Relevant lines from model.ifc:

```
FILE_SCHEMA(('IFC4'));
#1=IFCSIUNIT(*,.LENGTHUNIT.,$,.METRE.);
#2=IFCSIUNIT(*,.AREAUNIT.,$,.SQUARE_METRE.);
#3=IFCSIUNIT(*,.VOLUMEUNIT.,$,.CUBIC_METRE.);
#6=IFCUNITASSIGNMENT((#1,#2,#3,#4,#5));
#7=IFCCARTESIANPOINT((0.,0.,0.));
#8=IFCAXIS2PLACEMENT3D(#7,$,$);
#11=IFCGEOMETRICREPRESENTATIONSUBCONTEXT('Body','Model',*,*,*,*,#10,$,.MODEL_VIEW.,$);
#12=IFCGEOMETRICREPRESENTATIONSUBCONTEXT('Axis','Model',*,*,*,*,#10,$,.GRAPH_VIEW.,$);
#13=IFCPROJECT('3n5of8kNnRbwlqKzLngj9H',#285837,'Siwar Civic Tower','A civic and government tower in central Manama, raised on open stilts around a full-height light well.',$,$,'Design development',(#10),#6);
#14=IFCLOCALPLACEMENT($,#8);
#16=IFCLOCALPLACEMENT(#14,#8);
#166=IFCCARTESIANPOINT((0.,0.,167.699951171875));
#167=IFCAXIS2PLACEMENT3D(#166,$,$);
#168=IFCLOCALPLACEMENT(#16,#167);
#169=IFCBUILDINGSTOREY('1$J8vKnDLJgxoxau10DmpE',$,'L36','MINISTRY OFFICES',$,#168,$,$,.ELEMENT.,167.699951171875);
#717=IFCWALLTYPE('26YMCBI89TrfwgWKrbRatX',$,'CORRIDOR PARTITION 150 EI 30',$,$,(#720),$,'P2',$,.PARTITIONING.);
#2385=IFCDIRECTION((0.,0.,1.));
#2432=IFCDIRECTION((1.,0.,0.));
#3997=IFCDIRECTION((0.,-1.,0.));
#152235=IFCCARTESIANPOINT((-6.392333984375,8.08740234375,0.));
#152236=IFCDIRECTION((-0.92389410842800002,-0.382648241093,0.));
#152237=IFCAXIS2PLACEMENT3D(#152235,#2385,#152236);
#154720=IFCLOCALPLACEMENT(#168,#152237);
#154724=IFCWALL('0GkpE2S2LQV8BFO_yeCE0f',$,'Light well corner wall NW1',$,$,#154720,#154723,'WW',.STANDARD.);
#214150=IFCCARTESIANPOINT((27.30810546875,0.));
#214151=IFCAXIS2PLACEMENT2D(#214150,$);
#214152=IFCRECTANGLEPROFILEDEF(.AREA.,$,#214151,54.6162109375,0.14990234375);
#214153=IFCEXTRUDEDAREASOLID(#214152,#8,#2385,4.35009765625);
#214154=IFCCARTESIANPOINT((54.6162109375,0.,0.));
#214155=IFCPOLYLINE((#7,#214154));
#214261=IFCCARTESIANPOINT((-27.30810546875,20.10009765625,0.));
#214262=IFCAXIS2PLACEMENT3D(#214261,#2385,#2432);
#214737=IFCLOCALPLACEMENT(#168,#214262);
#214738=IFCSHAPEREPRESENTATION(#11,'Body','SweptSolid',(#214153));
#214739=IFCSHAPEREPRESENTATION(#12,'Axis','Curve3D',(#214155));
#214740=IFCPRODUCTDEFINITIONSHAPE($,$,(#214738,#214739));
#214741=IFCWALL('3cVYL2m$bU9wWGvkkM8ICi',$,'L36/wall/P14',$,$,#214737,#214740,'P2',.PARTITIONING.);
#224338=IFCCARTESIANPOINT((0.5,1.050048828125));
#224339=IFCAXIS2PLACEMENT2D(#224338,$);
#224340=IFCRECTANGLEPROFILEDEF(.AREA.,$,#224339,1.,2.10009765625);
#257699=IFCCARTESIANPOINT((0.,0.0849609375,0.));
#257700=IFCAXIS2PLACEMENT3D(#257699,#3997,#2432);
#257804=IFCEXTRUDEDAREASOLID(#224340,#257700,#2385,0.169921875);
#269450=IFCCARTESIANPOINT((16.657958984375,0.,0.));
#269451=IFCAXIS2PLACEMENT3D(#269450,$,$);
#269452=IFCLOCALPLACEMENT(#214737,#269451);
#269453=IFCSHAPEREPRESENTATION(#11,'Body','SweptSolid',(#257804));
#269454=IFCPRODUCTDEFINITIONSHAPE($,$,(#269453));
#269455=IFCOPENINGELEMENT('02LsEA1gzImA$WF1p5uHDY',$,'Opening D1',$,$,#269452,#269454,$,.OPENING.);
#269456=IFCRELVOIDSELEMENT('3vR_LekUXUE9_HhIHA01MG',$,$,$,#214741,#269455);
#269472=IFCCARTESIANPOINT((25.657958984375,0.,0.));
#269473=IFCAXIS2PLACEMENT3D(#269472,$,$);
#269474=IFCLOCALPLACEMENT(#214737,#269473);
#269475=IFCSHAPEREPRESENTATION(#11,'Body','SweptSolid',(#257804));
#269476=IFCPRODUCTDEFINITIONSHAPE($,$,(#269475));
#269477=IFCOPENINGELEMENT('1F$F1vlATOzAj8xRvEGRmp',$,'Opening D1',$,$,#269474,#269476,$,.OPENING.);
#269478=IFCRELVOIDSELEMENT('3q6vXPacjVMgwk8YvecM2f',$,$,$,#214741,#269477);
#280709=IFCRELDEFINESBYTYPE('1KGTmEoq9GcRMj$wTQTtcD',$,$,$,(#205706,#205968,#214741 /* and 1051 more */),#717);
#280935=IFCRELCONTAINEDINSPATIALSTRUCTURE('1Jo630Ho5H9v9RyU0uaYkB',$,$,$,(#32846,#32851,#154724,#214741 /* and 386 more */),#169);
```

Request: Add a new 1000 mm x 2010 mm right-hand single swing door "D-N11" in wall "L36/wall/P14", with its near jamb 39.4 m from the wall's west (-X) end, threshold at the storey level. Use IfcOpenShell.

```python
import numpy as np
import ifcopenshell
import ifcopenshell.api.feature
import ifcopenshell.api.geometry
import ifcopenshell.api.root
import ifcopenshell.api.spatial
import ifcopenshell.geom
import ifcopenshell.util.element
import ifcopenshell.util.placement
import ifcopenshell.util.representation
import ifcopenshell.util.shape
import ifcopenshell.util.unit

model = ifcopenshell.open("model.ifc")
unit_scale = ifcopenshell.util.unit.calculate_unit_scale(model)
settings = ifcopenshell.geom.settings()


def volume(element):
    """Net volume in cubic metres, openings subtracted."""
    shape = ifcopenshell.geom.create_shape(settings, element)
    return ifcopenshell.util.shape.get_volume(shape.geometry)


wall = model.by_guid("3cVYL2m$bU9wWGvkkM8ICi")
storey = ifcopenshell.util.element.get_container(wall, ifc_class="IfcBuildingStorey")
context = ifcopenshell.util.representation.get_context(model, "Model", "Body", "MODEL_VIEW")
before = volume(wall)

width, height, from_end, sill = 1, 2.01, 39.4, 0.0  # metres

# The wall runs along its own X axis, and the end named is its -X end.
wall_shape = ifcopenshell.geom.create_shape(settings, wall)
x, y, z = ifcopenshell.util.shape.get_vertices(wall_shape.geometry).T
start = x.min() + from_end
face, thickness = float(y.min()), float(y.max() - y.min())
wall_matrix = ifcopenshell.util.placement.get_local_placement(wall.ObjectPlacement)
level = ifcopenshell.util.placement.get_local_placement(storey.ObjectPlacement)[2, 3]


def in_wall(x, y):
    """Placement at x, y metres in the wall's axes, at sill height."""
    matrix = wall_matrix.copy()
    matrix[:, 3] = wall_matrix @ np.array([x / unit_scale, y / unit_scale, 0.0, 1.0])
    matrix[2, 3] = level + sill / unit_scale
    return matrix


# Opening: a box that overshoots both wall faces by 50 mm.
opening = ifcopenshell.api.root.create_entity(model, ifc_class="IfcOpeningElement", predefined_type="OPENING")
box = ifcopenshell.api.geometry.add_wall_representation(
    model, context=context, length=width, height=height, thickness=thickness + 0.1
)
ifcopenshell.api.geometry.assign_representation(model, product=opening, representation=box)
ifcopenshell.api.geometry.edit_object_placement(model, product=opening, matrix=in_wall(start, face - 0.05), is_si=False)
ifcopenshell.api.feature.add_feature(model, feature=opening, element=wall)

door = ifcopenshell.api.root.create_entity(model, ifc_class="IfcDoor", name="D-N11", predefined_type="DOOR")
door.OverallWidth, door.OverallHeight = width / unit_scale, height / unit_scale
door.OperationType = "SINGLE_SWING_RIGHT"
body = ifcopenshell.api.geometry.add_door_representation(
    model,
    context=context,
    overall_width=door.OverallWidth,
    overall_height=door.OverallHeight,
    operation_type="SINGLE_SWING_RIGHT",
    lining_properties={"LiningDepth": thickness / unit_scale, "ThresholdDepth": thickness / unit_scale},
)
ifcopenshell.api.geometry.assign_representation(model, product=door, representation=body)
ifcopenshell.api.spatial.assign_container(model, products=[door], relating_structure=storey)
ifcopenshell.api.feature.add_filling(model, opening=opening, element=door)

# The lining spans the wall, so the door starts at the wall face.
ifcopenshell.api.geometry.edit_object_placement(model, product=door, matrix=in_wall(start, face), is_si=False)

after = volume(wall)

print(f"wall volume {before:.3f} -> {after:.3f} m3")

model.write("model_edited.ifc")
```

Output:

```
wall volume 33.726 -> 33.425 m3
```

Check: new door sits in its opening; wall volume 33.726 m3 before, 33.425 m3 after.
